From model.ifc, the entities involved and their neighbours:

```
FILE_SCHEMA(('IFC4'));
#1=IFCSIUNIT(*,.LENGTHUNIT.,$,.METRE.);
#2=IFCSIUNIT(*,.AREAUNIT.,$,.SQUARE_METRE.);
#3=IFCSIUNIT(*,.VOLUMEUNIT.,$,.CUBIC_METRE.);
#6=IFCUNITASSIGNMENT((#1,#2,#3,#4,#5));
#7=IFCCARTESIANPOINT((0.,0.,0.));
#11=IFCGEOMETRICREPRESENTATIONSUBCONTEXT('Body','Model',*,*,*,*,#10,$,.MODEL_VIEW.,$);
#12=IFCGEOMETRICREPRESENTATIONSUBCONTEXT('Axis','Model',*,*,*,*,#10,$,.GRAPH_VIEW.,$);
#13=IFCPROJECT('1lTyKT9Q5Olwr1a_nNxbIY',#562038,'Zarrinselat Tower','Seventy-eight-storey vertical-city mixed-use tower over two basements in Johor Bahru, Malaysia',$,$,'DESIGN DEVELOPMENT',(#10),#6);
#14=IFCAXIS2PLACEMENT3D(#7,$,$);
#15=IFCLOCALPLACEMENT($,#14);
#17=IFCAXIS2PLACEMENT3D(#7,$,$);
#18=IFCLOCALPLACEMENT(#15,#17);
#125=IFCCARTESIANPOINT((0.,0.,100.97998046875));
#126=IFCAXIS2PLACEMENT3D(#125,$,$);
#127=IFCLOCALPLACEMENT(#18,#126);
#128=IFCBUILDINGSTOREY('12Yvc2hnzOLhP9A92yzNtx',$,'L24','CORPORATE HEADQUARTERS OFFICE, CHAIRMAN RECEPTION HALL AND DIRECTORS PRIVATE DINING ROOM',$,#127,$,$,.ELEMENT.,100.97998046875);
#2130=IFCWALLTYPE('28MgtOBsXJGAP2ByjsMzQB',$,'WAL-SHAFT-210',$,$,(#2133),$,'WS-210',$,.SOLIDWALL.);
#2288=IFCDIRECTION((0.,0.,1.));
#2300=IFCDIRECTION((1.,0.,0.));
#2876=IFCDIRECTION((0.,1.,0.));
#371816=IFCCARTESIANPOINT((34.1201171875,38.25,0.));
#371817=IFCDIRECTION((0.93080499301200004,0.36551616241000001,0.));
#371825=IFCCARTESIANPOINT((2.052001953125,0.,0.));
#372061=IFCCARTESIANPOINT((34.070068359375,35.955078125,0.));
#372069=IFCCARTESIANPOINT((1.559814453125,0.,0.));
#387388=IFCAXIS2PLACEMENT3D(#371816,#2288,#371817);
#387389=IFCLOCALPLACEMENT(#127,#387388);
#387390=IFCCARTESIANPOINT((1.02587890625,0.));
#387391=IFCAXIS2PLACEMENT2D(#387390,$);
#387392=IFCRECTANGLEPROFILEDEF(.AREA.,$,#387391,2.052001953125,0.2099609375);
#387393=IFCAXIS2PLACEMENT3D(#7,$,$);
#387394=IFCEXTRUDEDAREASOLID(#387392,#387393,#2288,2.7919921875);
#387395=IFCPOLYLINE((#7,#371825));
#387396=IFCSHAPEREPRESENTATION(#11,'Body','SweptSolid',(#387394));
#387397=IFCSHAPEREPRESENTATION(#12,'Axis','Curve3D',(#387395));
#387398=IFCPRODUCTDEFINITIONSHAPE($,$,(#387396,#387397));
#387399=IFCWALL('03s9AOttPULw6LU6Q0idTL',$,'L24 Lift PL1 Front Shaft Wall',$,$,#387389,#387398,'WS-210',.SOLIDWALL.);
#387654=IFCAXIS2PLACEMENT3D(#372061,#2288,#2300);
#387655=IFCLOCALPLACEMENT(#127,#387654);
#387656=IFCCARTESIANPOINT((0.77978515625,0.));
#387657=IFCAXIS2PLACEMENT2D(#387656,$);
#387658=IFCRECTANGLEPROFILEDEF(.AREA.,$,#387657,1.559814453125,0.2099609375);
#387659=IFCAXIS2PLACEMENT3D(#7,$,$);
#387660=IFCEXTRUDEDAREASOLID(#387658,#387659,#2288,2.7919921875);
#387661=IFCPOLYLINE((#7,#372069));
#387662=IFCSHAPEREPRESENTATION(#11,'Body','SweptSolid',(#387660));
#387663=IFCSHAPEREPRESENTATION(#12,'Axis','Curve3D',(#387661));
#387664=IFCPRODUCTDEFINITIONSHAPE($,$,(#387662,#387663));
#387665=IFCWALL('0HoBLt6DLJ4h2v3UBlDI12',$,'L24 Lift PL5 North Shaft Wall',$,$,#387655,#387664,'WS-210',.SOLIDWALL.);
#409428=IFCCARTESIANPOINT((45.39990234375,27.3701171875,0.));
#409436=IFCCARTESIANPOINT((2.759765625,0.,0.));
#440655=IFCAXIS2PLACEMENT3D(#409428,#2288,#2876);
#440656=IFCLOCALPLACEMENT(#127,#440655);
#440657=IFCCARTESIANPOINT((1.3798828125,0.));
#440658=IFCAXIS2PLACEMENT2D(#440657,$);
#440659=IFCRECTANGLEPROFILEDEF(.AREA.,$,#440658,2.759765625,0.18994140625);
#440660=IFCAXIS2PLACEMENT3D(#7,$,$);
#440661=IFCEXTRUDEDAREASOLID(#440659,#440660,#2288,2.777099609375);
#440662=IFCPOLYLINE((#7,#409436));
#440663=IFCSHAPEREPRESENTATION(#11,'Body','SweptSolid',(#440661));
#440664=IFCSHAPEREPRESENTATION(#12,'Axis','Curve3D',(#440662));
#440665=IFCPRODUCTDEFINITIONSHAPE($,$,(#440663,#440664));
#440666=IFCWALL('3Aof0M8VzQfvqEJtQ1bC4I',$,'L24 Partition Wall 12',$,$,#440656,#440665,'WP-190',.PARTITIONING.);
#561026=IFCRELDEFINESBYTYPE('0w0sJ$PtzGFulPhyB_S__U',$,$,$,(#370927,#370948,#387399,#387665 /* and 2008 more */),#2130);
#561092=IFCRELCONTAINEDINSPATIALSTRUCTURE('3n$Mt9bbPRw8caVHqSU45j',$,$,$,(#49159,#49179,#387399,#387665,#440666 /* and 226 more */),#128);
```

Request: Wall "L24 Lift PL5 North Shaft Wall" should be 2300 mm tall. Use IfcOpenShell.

```python
import ifcopenshell
import ifcopenshell.geom
import ifcopenshell.util.representation
import ifcopenshell.util.shape
import ifcopenshell.util.unit

model = ifcopenshell.open("model.ifc")
unit_scale = ifcopenshell.util.unit.calculate_unit_scale(model)
settings = ifcopenshell.geom.settings()


def volume(element):
    """Net volume in cubic metres, openings subtracted."""
    shape = ifcopenshell.geom.create_shape(settings, element)
    return ifcopenshell.util.shape.get_volume(shape.geometry)


wall = model.by_guid("0HoBLt6DLJ4h2v3UBlDI12")
before = volume(wall)

body = ifcopenshell.util.representation.get_representation(wall, "Model", "Body")
solid = body.Items[0]
old_height = solid.Depth
solid.Depth = 2.3 / unit_scale
after = volume(wall)

print(f"height {old_height:g} -> {solid.Depth:g}, volume {before:.3f} -> {after:.3f} m3")

model.write("model_rev.ifc")
```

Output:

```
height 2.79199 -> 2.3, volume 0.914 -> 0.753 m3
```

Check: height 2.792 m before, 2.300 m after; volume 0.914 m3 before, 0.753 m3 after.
